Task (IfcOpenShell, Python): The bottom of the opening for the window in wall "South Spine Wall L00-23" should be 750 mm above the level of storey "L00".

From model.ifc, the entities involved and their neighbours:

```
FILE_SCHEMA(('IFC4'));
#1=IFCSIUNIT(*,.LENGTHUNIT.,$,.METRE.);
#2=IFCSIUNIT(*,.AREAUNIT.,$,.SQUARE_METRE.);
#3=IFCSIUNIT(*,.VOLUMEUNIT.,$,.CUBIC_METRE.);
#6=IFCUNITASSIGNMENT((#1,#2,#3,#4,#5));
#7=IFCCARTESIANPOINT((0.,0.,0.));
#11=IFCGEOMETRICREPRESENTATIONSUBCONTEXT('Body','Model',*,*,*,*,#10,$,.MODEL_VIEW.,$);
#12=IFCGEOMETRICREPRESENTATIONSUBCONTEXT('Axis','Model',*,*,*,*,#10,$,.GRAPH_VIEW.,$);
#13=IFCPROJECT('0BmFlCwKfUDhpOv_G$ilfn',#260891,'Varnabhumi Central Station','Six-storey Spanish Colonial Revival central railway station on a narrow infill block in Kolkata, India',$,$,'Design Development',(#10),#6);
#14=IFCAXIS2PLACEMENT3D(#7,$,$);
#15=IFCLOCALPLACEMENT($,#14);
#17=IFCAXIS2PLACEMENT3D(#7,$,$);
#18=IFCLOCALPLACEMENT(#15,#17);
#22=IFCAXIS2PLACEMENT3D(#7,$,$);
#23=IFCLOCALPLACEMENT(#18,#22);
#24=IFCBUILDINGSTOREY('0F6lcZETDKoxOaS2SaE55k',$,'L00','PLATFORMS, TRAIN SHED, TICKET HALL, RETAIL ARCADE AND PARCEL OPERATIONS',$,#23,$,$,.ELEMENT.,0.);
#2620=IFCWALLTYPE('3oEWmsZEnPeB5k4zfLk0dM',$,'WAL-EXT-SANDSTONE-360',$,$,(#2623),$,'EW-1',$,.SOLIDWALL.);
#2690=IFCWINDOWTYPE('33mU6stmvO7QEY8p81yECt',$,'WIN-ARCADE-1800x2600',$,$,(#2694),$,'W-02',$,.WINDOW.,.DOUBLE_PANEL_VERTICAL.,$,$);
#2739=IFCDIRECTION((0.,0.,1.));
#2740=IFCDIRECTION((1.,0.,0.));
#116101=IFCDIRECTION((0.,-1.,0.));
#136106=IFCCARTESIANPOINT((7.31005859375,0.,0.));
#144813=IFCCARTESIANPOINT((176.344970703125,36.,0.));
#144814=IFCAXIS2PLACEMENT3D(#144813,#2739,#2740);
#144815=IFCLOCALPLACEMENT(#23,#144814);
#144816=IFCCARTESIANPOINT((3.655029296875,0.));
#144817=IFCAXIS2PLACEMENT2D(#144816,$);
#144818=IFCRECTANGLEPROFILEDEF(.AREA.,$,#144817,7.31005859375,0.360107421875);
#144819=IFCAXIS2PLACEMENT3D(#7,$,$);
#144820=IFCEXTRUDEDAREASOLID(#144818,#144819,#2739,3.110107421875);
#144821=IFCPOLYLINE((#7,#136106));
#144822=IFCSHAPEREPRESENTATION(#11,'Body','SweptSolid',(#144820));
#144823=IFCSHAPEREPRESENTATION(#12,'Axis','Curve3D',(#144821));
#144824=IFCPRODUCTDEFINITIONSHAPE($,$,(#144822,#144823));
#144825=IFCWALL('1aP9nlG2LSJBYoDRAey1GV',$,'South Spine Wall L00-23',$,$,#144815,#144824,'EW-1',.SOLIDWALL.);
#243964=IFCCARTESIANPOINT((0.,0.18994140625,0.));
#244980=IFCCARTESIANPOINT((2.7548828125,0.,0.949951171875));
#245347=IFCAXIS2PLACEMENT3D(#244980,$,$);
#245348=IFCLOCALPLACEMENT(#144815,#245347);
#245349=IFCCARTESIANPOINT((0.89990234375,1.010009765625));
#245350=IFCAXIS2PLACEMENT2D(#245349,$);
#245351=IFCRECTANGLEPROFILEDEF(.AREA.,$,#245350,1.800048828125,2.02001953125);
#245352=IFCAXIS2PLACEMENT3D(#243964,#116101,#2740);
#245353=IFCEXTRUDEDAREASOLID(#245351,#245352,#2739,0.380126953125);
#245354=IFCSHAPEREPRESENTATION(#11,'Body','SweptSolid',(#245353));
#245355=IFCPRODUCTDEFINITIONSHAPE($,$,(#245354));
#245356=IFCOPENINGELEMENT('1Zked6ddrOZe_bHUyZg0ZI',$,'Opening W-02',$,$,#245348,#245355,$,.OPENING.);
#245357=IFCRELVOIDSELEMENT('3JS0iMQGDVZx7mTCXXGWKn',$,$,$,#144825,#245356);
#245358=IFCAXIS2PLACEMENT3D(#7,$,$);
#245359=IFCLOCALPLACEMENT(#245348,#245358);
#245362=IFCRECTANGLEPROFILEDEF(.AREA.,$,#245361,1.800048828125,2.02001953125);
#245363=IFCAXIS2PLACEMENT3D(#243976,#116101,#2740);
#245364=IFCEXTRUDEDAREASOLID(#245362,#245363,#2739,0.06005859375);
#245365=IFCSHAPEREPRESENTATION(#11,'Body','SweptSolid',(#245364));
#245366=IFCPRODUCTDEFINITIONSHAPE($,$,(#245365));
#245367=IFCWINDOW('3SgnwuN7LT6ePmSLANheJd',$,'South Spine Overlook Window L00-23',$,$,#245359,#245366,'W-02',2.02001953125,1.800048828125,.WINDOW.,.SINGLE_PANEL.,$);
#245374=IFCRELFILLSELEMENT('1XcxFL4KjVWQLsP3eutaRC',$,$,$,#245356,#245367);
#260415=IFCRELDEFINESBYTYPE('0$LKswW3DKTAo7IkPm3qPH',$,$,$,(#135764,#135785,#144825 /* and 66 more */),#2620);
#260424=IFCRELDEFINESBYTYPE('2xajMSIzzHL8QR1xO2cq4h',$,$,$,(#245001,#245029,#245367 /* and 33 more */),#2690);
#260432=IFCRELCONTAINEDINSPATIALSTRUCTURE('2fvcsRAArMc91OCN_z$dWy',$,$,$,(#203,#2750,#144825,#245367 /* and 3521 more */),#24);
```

```python
import numpy as np
import ifcopenshell
import ifcopenshell.api.geometry
import ifcopenshell.geom
import ifcopenshell.util.element
import ifcopenshell.util.placement
import ifcopenshell.util.shape
import ifcopenshell.util.unit

model = ifcopenshell.open("model.ifc")
unit_scale = ifcopenshell.util.unit.calculate_unit_scale(model)

window = model.by_guid("3SgnwuN7LT6ePmSLANheJd")
opening = window.FillsVoids[0].RelatingOpeningElement
storey = ifcopenshell.util.element.get_container(window, ifc_class="IfcBuildingStorey")
level = ifcopenshell.util.placement.get_local_placement(storey.ObjectPlacement)[2, 3]

# The opening's origin need not be at the sill, so measure its lowest point.
shape = ifcopenshell.geom.create_shape(ifcopenshell.geom.settings(), opening)
bottom = ifcopenshell.util.shape.get_shape_bottom_elevation(shape, shape.geometry) / unit_scale
dz = level + 0.75 - bottom

shift = np.array([0.0, 0.0, dz])
# The window is placed relative to its opening, so it follows when the opening moves.
matrix = ifcopenshell.util.placement.get_local_placement(opening.ObjectPlacement)
matrix[:3, 3] += shift
ifcopenshell.api.geometry.edit_object_placement(
    model, product=opening, matrix=matrix, is_si=False, should_transform_children=True
)

print(f"moved by {dz * unit_scale:+.3f} m")

model.write("model_updated.ifc")
```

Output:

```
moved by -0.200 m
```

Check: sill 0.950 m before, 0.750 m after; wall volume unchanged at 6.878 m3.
